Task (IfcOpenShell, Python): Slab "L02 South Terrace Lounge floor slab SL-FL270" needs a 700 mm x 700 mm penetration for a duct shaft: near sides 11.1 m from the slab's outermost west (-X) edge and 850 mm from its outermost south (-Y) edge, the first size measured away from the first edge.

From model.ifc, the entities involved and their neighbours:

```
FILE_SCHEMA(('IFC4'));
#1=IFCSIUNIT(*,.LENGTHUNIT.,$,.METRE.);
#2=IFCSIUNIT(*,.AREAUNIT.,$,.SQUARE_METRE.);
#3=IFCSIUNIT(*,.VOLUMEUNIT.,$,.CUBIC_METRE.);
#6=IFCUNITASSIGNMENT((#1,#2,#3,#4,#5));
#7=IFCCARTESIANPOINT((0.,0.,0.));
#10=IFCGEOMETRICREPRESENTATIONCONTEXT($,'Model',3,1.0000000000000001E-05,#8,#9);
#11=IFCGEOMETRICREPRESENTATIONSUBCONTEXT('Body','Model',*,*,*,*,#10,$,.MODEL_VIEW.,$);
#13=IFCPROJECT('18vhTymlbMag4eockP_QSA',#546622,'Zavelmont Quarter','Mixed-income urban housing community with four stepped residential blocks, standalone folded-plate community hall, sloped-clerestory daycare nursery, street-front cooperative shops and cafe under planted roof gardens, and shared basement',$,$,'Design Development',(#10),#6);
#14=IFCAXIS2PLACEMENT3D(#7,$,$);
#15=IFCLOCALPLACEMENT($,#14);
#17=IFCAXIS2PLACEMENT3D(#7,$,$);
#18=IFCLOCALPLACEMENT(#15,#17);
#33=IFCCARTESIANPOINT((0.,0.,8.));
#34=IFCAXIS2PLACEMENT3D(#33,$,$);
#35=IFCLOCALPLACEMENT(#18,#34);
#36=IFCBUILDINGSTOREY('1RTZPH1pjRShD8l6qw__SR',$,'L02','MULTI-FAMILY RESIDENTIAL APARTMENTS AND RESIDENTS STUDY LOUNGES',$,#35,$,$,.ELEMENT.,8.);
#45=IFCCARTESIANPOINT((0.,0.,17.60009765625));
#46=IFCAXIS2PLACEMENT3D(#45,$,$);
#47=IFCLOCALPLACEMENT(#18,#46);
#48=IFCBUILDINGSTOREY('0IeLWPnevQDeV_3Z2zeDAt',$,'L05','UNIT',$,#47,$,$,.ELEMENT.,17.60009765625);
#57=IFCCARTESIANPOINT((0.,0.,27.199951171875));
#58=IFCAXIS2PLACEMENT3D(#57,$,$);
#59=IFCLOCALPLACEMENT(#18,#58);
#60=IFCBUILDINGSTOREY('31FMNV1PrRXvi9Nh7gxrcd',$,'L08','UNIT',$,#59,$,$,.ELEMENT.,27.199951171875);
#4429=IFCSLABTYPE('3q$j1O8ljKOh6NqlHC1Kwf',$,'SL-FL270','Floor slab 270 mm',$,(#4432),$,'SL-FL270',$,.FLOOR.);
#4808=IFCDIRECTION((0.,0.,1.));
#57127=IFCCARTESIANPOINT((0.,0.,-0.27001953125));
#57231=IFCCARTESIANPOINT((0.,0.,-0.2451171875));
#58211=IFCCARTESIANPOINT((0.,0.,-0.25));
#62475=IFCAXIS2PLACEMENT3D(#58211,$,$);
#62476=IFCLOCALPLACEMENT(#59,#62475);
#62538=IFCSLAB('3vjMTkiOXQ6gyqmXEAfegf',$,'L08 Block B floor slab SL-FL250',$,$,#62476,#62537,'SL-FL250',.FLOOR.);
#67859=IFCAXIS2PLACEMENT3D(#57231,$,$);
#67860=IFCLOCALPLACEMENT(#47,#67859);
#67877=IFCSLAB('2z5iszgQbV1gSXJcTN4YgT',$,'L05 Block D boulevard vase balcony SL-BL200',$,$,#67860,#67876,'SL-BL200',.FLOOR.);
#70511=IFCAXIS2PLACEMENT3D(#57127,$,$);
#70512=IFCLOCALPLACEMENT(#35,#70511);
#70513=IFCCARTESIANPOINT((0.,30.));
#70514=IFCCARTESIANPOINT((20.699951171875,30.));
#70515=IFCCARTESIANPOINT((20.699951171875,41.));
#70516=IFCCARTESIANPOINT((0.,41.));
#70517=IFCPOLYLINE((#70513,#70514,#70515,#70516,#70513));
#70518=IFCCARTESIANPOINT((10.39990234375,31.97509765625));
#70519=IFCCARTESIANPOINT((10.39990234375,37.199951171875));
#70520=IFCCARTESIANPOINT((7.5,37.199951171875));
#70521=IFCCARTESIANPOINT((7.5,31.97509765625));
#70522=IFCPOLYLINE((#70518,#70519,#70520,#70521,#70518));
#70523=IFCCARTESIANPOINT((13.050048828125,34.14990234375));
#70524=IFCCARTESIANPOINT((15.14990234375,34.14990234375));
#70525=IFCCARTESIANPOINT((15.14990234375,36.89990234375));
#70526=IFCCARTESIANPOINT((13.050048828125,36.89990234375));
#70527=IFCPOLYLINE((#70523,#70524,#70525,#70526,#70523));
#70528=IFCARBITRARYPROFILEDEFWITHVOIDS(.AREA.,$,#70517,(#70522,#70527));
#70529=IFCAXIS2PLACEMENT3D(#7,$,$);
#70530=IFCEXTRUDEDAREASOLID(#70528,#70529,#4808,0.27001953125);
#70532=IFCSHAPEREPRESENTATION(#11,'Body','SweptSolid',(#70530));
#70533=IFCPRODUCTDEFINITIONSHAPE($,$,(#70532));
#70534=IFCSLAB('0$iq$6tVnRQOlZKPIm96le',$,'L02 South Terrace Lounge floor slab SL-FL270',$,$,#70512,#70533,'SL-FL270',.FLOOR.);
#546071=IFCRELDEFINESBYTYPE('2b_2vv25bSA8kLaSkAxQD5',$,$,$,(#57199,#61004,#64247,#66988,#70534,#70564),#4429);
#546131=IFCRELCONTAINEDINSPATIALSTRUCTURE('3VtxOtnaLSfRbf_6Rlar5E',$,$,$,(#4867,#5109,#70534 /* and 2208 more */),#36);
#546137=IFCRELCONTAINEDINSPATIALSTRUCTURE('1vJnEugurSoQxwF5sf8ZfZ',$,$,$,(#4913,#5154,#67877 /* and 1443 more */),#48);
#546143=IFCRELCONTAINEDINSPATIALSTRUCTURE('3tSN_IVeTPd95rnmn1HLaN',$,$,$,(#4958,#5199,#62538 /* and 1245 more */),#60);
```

```python
import numpy as np
import ifcopenshell
import ifcopenshell.api.feature
import ifcopenshell.api.geometry
import ifcopenshell.api.root
import ifcopenshell.geom
import ifcopenshell.util.placement
import ifcopenshell.util.representation
import ifcopenshell.util.shape
import ifcopenshell.util.unit

model = ifcopenshell.open("model.ifc")
unit_scale = ifcopenshell.util.unit.calculate_unit_scale(model)
settings = ifcopenshell.geom.settings()


def volume(element):
    """Net volume in cubic metres, openings subtracted."""
    shape = ifcopenshell.geom.create_shape(settings, element)
    return ifcopenshell.util.shape.get_volume(shape.geometry)


slab = model.by_id(70534)
before = volume(slab)

# Extent in the slab's own axes, in metres. The edges named are its -X and -Y sides.
slab_shape = ifcopenshell.geom.create_shape(settings, slab)
vertices = ifcopenshell.util.shape.get_vertices(slab_shape.geometry)
x_min, y_min, bottom = vertices.min(axis=0)
top = vertices[:, 2].max()

opening = ifcopenshell.api.root.create_entity(model, ifc_class="IfcOpeningElement", name="Duct shaft opening", predefined_type="OPENING")
context = ifcopenshell.util.representation.get_context(model, "Model", "Body", "MODEL_VIEW")
width, depth = 0.7, 0.7
outline = [(0.0, 0.0), (width, 0.0), (width, depth), (0.0, depth), (0.0, 0.0)]
# Overshoot both faces by 50 mm so the cut is clean.
shape = ifcopenshell.api.geometry.add_slab_representation(
    model, context=context, depth=top - bottom + 0.1, polyline=outline
)
ifcopenshell.api.geometry.assign_representation(model, product=opening, representation=shape)

matrix = ifcopenshell.util.placement.get_local_placement(slab.ObjectPlacement)
matrix[:, 3] = matrix @ np.append(np.array([x_min + 11.1, y_min + 0.85, bottom - 0.05]) / unit_scale, 1.0)
ifcopenshell.api.geometry.edit_object_placement(model, product=opening, matrix=matrix, is_si=False)
ifcopenshell.api.feature.add_feature(model, feature=opening, element=slab)

after = volume(slab)

print(f"slab volume {before:.3f} -> {after:.3f} m3")

model.write("model_rev.ifc")
```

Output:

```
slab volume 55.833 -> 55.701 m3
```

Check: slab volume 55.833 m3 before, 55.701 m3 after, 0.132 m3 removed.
